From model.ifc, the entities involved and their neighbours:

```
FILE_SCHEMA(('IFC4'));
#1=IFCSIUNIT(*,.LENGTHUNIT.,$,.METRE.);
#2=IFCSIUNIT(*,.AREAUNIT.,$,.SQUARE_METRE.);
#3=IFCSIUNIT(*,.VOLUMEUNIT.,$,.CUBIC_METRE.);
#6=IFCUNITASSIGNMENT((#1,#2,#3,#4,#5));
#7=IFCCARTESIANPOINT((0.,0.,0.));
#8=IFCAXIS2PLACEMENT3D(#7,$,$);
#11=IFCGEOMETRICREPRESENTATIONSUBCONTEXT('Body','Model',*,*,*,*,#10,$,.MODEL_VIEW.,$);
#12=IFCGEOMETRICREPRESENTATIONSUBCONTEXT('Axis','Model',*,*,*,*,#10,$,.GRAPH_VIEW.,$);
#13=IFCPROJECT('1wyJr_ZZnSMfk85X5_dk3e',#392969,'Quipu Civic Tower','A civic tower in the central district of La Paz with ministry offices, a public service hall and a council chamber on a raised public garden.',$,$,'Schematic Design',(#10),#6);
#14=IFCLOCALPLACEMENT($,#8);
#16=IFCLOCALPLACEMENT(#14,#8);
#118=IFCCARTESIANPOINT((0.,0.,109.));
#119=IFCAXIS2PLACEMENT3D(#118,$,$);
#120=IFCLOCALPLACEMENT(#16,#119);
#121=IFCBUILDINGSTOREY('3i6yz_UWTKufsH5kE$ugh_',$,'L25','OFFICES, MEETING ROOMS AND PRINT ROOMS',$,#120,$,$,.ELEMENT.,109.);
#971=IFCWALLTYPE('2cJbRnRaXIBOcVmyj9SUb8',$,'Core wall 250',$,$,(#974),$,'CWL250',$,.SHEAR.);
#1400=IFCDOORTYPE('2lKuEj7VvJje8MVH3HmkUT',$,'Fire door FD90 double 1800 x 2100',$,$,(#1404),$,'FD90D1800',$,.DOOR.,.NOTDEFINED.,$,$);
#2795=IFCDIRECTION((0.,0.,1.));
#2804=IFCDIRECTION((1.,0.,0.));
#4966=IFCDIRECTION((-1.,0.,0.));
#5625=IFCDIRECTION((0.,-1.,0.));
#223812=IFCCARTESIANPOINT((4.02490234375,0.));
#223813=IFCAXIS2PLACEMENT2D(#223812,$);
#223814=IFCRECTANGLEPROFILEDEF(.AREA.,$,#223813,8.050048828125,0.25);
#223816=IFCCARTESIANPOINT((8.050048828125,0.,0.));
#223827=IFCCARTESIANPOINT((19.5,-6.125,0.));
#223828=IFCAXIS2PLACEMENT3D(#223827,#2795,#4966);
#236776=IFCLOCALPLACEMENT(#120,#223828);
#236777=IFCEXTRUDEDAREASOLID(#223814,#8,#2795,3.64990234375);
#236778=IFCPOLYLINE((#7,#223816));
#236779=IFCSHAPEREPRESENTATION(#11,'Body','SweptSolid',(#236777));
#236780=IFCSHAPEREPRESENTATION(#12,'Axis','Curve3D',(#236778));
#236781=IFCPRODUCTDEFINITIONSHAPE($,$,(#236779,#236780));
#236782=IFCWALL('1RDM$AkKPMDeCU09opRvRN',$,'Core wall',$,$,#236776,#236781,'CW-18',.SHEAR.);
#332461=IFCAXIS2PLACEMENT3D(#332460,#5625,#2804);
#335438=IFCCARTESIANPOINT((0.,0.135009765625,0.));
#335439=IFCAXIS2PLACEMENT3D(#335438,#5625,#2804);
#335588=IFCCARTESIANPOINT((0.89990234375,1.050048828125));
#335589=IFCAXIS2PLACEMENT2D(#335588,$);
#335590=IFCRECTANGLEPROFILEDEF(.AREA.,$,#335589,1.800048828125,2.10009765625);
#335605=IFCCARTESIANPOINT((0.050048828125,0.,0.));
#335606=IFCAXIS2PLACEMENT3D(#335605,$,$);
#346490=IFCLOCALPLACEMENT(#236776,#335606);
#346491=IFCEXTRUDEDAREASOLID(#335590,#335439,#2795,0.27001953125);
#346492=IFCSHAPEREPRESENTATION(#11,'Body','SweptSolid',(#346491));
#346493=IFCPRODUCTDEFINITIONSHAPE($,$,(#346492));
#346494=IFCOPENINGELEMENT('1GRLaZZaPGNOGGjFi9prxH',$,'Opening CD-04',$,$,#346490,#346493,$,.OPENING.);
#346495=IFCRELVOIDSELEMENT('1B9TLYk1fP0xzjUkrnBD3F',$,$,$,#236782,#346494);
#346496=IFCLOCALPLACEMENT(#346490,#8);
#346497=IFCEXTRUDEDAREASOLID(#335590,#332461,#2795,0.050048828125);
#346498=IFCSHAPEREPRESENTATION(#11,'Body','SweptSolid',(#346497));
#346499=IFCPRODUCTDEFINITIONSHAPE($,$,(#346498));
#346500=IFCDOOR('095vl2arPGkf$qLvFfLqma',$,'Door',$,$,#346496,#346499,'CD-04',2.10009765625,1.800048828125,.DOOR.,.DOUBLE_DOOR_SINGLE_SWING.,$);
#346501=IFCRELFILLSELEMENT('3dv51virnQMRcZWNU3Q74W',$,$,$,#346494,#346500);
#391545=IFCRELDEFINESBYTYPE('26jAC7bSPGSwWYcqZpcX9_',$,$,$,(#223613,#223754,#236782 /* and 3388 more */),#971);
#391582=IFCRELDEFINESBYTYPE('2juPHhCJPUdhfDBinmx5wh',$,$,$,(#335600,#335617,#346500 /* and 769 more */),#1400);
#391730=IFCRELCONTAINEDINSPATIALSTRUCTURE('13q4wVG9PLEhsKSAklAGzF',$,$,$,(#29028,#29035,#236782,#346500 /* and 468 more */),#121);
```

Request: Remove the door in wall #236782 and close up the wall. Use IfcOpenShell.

```python
import ifcopenshell
import ifcopenshell.api.feature
import ifcopenshell.api.root
import ifcopenshell.geom
import ifcopenshell.util.shape

model = ifcopenshell.open("model.ifc")
settings = ifcopenshell.geom.settings()


def volume(element):
    """Net volume in cubic metres, openings subtracted."""
    shape = ifcopenshell.geom.create_shape(settings, element)
    return ifcopenshell.util.shape.get_volume(shape.geometry)


door = model.by_guid("095vl2arPGkf$qLvFfLqma")
opening = door.FillsVoids[0].RelatingOpeningElement
wall = opening.VoidsElements[0].RelatingBuildingElement
before = volume(wall)

ifcopenshell.api.root.remove_product(model, product=door)
ifcopenshell.api.feature.remove_feature(model, feature=opening)

after = volume(wall)

print(f"wall volume {before:.3f} -> {after:.3f} m3")

model.write("model_updated.ifc")
```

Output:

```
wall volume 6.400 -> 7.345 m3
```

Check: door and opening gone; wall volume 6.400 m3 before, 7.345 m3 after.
